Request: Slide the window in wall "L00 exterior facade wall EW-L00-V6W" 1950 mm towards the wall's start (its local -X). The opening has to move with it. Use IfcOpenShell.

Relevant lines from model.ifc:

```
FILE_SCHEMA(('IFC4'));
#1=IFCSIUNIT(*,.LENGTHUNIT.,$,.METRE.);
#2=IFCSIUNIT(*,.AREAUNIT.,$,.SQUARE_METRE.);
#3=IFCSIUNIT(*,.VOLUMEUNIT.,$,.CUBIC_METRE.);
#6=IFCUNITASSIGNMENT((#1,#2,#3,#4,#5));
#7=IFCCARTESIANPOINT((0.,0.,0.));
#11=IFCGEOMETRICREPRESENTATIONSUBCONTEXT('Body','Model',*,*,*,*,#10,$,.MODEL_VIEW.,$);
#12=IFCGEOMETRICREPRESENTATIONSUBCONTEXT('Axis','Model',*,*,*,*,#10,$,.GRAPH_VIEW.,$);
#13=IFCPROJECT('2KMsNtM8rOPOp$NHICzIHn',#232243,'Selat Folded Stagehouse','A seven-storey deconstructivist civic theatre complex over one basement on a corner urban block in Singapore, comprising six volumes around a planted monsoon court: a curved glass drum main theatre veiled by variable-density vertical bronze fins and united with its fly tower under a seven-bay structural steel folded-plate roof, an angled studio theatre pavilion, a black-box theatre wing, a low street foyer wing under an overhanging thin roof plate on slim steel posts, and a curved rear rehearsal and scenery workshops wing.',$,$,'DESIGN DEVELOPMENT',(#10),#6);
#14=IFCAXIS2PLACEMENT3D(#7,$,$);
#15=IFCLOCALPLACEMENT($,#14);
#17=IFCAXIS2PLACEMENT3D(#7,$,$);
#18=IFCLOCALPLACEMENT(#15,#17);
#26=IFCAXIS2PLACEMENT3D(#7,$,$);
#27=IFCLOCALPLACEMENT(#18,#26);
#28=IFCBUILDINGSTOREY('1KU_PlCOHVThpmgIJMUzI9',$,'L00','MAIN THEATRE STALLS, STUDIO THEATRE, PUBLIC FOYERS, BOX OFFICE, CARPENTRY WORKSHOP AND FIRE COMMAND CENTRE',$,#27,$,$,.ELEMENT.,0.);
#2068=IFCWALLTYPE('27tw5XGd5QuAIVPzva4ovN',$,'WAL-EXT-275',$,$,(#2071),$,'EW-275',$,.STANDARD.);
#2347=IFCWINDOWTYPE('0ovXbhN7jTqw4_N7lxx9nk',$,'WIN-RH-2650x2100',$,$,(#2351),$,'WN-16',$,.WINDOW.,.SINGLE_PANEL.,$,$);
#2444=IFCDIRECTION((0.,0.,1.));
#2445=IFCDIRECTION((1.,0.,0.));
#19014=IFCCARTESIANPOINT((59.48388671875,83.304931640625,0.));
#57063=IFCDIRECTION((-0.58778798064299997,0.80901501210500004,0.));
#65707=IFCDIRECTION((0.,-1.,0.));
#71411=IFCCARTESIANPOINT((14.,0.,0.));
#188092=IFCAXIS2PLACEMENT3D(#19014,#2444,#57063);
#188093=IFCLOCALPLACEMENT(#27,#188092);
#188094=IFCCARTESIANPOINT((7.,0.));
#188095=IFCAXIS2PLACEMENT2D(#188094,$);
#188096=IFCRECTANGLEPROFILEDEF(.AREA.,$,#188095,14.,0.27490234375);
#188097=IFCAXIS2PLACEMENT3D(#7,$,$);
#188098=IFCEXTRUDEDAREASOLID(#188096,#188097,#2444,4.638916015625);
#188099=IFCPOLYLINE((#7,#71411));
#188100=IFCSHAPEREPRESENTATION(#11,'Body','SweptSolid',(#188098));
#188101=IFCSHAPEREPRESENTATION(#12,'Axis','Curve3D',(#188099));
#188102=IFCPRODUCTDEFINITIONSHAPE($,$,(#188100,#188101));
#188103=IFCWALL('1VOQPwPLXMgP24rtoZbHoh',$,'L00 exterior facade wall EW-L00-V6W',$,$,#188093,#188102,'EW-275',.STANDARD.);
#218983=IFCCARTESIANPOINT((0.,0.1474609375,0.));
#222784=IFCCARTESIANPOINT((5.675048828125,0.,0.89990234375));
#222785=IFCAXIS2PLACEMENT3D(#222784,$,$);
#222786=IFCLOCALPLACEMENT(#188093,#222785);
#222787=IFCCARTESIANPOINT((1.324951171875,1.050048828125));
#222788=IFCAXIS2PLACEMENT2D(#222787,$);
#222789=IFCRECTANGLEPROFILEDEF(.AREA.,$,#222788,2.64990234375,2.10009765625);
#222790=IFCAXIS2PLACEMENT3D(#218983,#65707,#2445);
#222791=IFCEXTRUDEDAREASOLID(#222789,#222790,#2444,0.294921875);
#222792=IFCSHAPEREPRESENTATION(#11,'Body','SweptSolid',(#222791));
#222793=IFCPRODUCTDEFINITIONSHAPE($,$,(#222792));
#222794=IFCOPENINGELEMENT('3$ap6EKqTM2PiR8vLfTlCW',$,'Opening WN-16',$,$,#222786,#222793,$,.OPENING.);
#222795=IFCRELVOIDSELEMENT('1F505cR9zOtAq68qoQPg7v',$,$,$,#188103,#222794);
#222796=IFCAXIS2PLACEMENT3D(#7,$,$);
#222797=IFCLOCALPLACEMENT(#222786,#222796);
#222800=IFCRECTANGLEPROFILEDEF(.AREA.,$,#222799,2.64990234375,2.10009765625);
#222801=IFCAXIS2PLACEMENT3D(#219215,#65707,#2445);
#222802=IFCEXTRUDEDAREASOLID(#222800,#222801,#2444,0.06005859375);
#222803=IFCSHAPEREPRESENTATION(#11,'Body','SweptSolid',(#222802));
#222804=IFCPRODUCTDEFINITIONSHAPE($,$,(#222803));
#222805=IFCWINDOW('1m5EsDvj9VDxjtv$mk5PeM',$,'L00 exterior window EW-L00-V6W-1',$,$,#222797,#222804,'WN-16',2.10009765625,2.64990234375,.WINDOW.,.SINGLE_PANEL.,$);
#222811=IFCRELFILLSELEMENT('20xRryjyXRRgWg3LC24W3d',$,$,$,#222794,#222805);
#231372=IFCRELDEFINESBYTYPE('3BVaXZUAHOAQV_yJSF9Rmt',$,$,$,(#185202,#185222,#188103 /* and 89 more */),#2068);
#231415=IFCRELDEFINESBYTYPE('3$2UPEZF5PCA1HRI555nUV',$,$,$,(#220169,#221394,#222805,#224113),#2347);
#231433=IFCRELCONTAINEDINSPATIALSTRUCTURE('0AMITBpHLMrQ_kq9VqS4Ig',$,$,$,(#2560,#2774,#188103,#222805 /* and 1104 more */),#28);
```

```python
import ifcopenshell
import ifcopenshell.api.geometry
import ifcopenshell.util.placement
import ifcopenshell.util.unit

model = ifcopenshell.open("model.ifc")
unit_scale = ifcopenshell.util.unit.calculate_unit_scale(model)

window = model.by_id(222805)
opening = window.FillsVoids[0].RelatingOpeningElement
wall = opening.VoidsElements[0].RelatingBuildingElement

wall_matrix = ifcopenshell.util.placement.get_local_placement(wall.ObjectPlacement)
shift = wall_matrix[:3, 0] * -1.95 / unit_scale
before = ifcopenshell.util.placement.get_local_placement(window.ObjectPlacement)[:3, 3].copy()

# The window is placed relative to its opening, so it follows when the opening moves.
matrix = ifcopenshell.util.placement.get_local_placement(opening.ObjectPlacement)
matrix[:3, 3] += shift
ifcopenshell.api.geometry.edit_object_placement(
    model, product=opening, matrix=matrix, is_si=False, should_transform_children=True
)

after = ifcopenshell.util.placement.get_local_placement(window.ObjectPlacement)[:3, 3]
print("window moved by", (after - before).round(3) + 0.0)

model.write("model_v2.ifc")
```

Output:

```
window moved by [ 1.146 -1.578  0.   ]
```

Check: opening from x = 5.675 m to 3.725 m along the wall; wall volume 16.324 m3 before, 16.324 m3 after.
